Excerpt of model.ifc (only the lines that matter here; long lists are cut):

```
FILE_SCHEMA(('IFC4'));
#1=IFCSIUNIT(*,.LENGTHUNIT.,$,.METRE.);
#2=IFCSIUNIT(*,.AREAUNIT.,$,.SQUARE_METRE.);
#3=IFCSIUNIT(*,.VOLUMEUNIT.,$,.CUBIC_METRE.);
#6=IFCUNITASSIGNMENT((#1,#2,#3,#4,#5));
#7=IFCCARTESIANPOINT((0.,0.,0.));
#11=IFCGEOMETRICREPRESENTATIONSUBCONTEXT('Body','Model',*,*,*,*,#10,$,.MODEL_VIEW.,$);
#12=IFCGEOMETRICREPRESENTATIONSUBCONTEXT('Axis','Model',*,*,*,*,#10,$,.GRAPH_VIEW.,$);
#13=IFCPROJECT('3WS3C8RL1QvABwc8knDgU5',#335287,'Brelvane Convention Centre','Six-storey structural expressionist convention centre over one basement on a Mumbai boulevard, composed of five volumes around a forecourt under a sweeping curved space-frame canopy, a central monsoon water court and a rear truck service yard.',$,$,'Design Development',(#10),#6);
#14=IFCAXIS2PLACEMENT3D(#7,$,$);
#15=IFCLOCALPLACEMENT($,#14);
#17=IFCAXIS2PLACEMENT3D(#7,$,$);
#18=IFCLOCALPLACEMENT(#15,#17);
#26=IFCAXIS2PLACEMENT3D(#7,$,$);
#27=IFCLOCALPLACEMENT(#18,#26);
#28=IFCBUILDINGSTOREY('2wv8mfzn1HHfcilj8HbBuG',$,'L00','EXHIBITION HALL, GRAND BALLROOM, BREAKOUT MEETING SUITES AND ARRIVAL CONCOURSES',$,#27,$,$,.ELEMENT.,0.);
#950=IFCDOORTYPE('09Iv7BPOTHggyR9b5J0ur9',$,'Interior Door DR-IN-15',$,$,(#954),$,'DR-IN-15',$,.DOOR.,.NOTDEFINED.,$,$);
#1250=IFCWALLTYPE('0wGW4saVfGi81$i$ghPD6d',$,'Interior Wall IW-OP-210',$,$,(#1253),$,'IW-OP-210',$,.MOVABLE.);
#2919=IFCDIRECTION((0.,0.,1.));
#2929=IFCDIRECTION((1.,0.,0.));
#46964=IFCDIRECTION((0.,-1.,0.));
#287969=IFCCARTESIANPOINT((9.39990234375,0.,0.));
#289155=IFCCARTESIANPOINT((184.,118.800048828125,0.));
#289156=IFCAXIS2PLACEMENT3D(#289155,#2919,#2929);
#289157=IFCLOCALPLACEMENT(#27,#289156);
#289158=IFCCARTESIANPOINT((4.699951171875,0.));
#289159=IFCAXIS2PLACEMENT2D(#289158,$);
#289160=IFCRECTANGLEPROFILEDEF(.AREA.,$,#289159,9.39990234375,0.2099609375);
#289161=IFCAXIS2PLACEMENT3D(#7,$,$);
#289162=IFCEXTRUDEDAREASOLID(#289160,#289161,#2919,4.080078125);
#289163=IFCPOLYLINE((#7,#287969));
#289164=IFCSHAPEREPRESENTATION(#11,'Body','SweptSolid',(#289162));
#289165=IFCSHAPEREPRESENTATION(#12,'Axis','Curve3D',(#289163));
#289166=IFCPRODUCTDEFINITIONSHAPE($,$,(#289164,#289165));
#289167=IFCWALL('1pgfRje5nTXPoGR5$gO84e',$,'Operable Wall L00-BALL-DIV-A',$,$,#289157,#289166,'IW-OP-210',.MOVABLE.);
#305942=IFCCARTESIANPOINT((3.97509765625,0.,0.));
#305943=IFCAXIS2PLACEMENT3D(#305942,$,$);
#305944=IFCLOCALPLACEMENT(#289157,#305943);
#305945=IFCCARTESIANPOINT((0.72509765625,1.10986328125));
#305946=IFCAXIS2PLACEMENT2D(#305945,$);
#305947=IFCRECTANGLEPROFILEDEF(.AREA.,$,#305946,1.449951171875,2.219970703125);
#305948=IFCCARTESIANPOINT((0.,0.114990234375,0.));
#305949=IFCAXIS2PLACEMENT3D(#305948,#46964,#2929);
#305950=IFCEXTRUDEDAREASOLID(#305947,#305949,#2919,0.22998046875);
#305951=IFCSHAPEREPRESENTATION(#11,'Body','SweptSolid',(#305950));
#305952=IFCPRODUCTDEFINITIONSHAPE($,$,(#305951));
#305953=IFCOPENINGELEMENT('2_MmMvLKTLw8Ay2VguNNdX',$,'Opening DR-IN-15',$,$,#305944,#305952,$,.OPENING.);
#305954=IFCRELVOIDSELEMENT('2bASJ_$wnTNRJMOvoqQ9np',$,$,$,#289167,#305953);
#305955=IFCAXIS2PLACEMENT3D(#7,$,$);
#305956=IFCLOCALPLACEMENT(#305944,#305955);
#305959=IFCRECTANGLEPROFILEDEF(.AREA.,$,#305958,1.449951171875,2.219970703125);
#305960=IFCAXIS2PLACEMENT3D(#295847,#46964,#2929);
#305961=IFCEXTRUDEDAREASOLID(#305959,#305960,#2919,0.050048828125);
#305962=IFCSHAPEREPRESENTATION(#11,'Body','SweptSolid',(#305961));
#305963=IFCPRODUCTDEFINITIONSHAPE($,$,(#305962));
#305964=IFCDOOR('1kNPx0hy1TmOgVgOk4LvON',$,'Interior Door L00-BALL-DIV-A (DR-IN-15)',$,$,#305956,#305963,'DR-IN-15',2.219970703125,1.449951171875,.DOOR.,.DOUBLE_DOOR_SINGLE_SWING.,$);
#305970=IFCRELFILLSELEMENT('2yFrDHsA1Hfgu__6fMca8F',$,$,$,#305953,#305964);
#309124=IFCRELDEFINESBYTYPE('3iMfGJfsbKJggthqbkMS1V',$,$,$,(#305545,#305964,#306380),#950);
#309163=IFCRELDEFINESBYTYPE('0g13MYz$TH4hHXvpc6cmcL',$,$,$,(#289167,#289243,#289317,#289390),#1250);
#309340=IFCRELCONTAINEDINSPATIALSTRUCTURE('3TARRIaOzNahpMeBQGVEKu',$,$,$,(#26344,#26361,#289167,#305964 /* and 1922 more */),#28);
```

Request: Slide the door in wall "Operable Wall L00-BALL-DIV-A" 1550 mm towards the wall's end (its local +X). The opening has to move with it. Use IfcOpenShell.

```python
import ifcopenshell
import ifcopenshell.api.geometry
import ifcopenshell.util.placement

model = ifcopenshell.open("model.ifc")

door = model.by_guid("1kNPx0hy1TmOgVgOk4LvON")
opening = door.FillsVoids[0].RelatingOpeningElement
wall = opening.VoidsElements[0].RelatingBuildingElement

wall_matrix = ifcopenshell.util.placement.get_local_placement(wall.ObjectPlacement)
shift = wall_matrix[:3, 0] * 1.55
before = ifcopenshell.util.placement.get_local_placement(door.ObjectPlacement)[:3, 3].copy()

# The door is placed relative to its opening, so it follows when the opening moves.
matrix = ifcopenshell.util.placement.get_local_placement(opening.ObjectPlacement)
matrix[:3, 3] += shift
ifcopenshell.api.geometry.edit_object_placement(
    model, product=opening, matrix=matrix, is_si=False, should_transform_children=True
)

after = ifcopenshell.util.placement.get_local_placement(door.ObjectPlacement)[:3, 3]
print("door moved by", (after - before).round(3) + 0.0)

model.write("model_v2.ifc")
```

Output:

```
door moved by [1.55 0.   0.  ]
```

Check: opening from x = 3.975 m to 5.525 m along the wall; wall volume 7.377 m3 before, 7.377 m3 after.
